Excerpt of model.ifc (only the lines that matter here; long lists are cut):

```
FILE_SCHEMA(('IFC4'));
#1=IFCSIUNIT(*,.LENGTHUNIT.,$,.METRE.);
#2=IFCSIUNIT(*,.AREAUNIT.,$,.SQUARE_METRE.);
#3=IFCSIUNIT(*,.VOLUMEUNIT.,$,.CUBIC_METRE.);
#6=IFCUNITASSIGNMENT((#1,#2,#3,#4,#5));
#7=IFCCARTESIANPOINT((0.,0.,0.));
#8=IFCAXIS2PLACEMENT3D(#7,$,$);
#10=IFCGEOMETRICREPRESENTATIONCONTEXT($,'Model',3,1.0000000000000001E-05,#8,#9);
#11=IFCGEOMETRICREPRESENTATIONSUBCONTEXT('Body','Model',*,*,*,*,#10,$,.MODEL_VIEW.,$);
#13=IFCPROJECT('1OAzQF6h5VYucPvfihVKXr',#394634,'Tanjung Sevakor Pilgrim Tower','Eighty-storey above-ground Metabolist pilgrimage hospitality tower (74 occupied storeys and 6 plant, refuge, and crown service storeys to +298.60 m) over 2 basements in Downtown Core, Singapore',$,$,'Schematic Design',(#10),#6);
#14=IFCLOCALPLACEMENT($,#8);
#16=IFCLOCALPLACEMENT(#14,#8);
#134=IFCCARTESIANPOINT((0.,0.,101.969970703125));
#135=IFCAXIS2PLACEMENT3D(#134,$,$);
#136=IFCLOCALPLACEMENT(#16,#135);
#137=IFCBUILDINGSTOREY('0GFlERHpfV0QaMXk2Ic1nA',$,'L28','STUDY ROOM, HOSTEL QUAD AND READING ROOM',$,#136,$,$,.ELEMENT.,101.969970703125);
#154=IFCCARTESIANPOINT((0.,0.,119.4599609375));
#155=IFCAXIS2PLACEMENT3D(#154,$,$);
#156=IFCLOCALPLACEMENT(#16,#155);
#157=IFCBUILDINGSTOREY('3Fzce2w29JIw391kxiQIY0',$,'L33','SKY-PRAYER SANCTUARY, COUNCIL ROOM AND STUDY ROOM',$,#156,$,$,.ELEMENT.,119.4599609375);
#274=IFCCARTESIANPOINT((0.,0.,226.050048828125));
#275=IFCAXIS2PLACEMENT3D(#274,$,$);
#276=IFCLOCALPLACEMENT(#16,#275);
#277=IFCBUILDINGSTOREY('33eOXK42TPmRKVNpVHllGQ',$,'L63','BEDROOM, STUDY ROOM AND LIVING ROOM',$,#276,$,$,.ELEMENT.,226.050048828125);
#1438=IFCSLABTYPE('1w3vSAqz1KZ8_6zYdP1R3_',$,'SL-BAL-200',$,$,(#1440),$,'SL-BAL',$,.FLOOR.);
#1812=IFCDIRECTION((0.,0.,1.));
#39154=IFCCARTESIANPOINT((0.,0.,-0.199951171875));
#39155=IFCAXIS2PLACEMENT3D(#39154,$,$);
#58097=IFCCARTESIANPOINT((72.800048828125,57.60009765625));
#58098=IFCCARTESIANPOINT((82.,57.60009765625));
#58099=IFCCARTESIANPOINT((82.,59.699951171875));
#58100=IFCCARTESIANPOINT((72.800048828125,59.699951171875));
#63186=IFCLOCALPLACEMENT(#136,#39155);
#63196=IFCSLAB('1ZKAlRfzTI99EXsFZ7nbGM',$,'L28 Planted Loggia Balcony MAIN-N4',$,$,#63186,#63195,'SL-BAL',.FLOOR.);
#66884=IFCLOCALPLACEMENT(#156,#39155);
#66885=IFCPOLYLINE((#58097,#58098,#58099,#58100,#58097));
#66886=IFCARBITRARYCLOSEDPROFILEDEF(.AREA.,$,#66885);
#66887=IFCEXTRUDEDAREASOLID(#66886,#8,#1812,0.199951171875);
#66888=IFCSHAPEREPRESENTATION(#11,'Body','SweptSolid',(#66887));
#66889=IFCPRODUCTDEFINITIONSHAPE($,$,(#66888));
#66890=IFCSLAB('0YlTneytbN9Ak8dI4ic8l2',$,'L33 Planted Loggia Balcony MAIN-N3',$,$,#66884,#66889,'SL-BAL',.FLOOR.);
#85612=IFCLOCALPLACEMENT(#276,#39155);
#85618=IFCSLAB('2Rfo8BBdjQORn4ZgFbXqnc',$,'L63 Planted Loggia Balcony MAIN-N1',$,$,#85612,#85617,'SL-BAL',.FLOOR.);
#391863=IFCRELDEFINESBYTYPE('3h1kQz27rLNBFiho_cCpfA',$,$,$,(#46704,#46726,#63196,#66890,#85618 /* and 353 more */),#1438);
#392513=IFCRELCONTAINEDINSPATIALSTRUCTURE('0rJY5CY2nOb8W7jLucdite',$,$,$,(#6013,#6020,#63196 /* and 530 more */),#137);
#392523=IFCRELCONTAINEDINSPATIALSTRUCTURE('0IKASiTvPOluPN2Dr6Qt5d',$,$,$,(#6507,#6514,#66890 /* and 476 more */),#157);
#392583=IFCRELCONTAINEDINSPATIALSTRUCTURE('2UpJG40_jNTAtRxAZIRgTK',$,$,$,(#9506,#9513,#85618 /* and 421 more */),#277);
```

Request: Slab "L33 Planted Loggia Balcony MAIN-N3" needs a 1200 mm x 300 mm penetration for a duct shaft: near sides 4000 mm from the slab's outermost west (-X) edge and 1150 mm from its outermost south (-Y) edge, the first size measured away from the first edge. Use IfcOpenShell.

```python
import numpy as np
import ifcopenshell
import ifcopenshell.api.feature
import ifcopenshell.api.geometry
import ifcopenshell.api.root
import ifcopenshell.geom
import ifcopenshell.util.placement
import ifcopenshell.util.representation
import ifcopenshell.util.shape
import ifcopenshell.util.unit

model = ifcopenshell.open("model.ifc")
unit_scale = ifcopenshell.util.unit.calculate_unit_scale(model)
settings = ifcopenshell.geom.settings()


def volume(element):
    """Net volume in cubic metres, openings subtracted."""
    shape = ifcopenshell.geom.create_shape(settings, element)
    return ifcopenshell.util.shape.get_volume(shape.geometry)


slab = model.by_guid("0YlTneytbN9Ak8dI4ic8l2")
before = volume(slab)

# Extent in the slab's own axes, in metres. The edges named are its -X and -Y sides.
slab_shape = ifcopenshell.geom.create_shape(settings, slab)
vertices = ifcopenshell.util.shape.get_vertices(slab_shape.geometry)
x_min, y_min, bottom = vertices.min(axis=0)
top = vertices[:, 2].max()

opening = ifcopenshell.api.root.create_entity(model, ifc_class="IfcOpeningElement", name="Duct shaft opening", predefined_type="OPENING")
context = ifcopenshell.util.representation.get_context(model, "Model", "Body", "MODEL_VIEW")
width, depth = 1.2, 0.3
outline = [(0.0, 0.0), (width, 0.0), (width, depth), (0.0, depth), (0.0, 0.0)]
# Overshoot both faces by 50 mm so the cut is clean.
shape = ifcopenshell.api.geometry.add_slab_representation(
    model, context=context, depth=top - bottom + 0.1, polyline=outline
)
ifcopenshell.api.geometry.assign_representation(model, product=opening, representation=shape)

matrix = ifcopenshell.util.placement.get_local_placement(slab.ObjectPlacement)
matrix[:, 3] = matrix @ np.append(np.array([x_min + 4, y_min + 1.15, bottom - 0.05]) / unit_scale, 1.0)
ifcopenshell.api.geometry.edit_object_placement(model, product=opening, matrix=matrix, is_si=False)
ifcopenshell.api.feature.add_feature(model, feature=opening, element=slab)

after = volume(slab)

print(f"slab volume {before:.3f} -> {after:.3f} m3")

model.write("model-out.ifc")
```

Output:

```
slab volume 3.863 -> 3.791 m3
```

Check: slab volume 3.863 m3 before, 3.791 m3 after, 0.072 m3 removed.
